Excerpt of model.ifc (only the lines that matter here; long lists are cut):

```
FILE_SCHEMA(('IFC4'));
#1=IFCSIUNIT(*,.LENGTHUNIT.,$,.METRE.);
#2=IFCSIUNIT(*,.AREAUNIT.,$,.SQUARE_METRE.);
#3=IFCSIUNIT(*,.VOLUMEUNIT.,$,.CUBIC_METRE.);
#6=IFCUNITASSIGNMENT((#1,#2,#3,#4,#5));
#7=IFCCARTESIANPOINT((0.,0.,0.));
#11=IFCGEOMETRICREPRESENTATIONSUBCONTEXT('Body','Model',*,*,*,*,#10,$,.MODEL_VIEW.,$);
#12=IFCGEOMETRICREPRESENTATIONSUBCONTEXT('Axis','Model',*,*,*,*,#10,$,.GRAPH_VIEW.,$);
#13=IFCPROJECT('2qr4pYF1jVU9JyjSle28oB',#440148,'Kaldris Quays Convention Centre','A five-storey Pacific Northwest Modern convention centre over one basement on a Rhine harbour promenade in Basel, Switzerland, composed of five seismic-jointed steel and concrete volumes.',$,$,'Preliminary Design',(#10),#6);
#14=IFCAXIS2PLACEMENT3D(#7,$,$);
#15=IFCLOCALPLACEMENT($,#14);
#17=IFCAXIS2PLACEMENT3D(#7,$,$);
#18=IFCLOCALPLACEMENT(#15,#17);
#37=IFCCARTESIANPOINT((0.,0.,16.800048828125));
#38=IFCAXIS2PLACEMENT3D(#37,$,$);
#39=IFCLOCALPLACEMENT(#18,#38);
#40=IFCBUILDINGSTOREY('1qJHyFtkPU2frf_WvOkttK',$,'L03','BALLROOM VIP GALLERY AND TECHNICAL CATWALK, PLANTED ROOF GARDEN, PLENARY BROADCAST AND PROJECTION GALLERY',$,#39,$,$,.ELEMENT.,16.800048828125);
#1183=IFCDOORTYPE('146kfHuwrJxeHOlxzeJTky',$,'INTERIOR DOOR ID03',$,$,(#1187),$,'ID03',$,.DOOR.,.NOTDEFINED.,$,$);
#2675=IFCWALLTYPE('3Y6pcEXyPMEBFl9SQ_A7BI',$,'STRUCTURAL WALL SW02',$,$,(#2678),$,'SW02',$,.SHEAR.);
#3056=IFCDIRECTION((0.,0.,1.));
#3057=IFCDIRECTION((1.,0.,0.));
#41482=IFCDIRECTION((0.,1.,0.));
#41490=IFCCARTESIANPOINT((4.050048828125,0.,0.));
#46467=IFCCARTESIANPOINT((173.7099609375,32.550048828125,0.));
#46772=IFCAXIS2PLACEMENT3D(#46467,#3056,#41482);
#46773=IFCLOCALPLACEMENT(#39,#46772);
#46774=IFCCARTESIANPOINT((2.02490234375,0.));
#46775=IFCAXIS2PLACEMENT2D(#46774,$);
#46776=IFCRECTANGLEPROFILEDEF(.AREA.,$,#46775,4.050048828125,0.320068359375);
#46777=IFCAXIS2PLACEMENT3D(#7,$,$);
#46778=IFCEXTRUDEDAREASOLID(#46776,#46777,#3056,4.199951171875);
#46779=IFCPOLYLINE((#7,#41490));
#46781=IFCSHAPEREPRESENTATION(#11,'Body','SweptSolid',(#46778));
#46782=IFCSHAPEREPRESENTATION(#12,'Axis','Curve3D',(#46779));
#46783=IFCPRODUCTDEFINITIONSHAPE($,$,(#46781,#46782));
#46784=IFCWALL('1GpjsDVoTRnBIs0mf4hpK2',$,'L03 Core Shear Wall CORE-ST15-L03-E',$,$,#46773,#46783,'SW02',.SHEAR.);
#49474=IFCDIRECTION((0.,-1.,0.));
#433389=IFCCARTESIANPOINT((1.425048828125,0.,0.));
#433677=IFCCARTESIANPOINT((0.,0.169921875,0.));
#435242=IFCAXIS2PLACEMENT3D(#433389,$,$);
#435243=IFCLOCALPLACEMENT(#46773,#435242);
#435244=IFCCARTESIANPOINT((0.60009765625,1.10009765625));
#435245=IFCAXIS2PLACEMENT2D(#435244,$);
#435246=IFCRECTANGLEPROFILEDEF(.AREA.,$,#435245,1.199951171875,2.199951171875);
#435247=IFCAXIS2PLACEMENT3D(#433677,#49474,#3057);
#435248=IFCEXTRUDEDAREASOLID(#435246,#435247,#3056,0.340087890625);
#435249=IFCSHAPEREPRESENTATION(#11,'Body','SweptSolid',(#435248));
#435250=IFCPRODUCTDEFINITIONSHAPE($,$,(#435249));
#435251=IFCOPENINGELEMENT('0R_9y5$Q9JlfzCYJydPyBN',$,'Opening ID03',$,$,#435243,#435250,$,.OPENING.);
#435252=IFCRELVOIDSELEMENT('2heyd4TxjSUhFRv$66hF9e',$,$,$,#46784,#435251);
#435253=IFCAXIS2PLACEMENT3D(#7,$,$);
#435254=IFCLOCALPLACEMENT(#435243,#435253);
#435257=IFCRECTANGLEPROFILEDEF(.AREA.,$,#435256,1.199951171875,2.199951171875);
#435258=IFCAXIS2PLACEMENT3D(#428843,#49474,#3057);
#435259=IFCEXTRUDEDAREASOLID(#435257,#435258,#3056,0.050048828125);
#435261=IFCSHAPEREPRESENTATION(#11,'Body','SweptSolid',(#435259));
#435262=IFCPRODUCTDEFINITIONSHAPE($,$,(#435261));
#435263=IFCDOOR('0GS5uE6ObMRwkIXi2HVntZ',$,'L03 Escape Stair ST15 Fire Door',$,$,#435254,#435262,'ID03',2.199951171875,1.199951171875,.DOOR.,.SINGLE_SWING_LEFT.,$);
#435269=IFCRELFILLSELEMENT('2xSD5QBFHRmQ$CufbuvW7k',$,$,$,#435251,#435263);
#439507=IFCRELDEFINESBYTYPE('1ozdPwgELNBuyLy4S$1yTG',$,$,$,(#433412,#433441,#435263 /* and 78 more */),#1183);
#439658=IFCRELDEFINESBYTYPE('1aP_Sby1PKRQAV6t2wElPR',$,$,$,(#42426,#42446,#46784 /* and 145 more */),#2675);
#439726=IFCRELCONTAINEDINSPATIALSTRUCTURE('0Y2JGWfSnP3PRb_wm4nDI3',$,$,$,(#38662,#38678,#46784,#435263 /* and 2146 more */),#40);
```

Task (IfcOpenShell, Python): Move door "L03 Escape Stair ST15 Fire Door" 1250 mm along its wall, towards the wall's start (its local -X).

```python
import ifcopenshell
import ifcopenshell.api.geometry
import ifcopenshell.util.placement
import ifcopenshell.util.unit

model = ifcopenshell.open("model.ifc")
unit_scale = ifcopenshell.util.unit.calculate_unit_scale(model)

door = model.by_guid("0GS5uE6ObMRwkIXi2HVntZ")
opening = door.FillsVoids[0].RelatingOpeningElement
wall = opening.VoidsElements[0].RelatingBuildingElement

wall_matrix = ifcopenshell.util.placement.get_local_placement(wall.ObjectPlacement)
shift = wall_matrix[:3, 0] * -1.25 / unit_scale
before = ifcopenshell.util.placement.get_local_placement(door.ObjectPlacement)[:3, 3].copy()

# The door is placed relative to its opening, so it follows when the opening moves.
matrix = ifcopenshell.util.placement.get_local_placement(opening.ObjectPlacement)
matrix[:3, 3] += shift
ifcopenshell.api.geometry.edit_object_placement(
    model, product=opening, matrix=matrix, is_si=False, should_transform_children=True
)

after = ifcopenshell.util.placement.get_local_placement(door.ObjectPlacement)[:3, 3]
print("door moved by", (after - before).round(3) + 0.0)

model.write("model_v2.ifc")
```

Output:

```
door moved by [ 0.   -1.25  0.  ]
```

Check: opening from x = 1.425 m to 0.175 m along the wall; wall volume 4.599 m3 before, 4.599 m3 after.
